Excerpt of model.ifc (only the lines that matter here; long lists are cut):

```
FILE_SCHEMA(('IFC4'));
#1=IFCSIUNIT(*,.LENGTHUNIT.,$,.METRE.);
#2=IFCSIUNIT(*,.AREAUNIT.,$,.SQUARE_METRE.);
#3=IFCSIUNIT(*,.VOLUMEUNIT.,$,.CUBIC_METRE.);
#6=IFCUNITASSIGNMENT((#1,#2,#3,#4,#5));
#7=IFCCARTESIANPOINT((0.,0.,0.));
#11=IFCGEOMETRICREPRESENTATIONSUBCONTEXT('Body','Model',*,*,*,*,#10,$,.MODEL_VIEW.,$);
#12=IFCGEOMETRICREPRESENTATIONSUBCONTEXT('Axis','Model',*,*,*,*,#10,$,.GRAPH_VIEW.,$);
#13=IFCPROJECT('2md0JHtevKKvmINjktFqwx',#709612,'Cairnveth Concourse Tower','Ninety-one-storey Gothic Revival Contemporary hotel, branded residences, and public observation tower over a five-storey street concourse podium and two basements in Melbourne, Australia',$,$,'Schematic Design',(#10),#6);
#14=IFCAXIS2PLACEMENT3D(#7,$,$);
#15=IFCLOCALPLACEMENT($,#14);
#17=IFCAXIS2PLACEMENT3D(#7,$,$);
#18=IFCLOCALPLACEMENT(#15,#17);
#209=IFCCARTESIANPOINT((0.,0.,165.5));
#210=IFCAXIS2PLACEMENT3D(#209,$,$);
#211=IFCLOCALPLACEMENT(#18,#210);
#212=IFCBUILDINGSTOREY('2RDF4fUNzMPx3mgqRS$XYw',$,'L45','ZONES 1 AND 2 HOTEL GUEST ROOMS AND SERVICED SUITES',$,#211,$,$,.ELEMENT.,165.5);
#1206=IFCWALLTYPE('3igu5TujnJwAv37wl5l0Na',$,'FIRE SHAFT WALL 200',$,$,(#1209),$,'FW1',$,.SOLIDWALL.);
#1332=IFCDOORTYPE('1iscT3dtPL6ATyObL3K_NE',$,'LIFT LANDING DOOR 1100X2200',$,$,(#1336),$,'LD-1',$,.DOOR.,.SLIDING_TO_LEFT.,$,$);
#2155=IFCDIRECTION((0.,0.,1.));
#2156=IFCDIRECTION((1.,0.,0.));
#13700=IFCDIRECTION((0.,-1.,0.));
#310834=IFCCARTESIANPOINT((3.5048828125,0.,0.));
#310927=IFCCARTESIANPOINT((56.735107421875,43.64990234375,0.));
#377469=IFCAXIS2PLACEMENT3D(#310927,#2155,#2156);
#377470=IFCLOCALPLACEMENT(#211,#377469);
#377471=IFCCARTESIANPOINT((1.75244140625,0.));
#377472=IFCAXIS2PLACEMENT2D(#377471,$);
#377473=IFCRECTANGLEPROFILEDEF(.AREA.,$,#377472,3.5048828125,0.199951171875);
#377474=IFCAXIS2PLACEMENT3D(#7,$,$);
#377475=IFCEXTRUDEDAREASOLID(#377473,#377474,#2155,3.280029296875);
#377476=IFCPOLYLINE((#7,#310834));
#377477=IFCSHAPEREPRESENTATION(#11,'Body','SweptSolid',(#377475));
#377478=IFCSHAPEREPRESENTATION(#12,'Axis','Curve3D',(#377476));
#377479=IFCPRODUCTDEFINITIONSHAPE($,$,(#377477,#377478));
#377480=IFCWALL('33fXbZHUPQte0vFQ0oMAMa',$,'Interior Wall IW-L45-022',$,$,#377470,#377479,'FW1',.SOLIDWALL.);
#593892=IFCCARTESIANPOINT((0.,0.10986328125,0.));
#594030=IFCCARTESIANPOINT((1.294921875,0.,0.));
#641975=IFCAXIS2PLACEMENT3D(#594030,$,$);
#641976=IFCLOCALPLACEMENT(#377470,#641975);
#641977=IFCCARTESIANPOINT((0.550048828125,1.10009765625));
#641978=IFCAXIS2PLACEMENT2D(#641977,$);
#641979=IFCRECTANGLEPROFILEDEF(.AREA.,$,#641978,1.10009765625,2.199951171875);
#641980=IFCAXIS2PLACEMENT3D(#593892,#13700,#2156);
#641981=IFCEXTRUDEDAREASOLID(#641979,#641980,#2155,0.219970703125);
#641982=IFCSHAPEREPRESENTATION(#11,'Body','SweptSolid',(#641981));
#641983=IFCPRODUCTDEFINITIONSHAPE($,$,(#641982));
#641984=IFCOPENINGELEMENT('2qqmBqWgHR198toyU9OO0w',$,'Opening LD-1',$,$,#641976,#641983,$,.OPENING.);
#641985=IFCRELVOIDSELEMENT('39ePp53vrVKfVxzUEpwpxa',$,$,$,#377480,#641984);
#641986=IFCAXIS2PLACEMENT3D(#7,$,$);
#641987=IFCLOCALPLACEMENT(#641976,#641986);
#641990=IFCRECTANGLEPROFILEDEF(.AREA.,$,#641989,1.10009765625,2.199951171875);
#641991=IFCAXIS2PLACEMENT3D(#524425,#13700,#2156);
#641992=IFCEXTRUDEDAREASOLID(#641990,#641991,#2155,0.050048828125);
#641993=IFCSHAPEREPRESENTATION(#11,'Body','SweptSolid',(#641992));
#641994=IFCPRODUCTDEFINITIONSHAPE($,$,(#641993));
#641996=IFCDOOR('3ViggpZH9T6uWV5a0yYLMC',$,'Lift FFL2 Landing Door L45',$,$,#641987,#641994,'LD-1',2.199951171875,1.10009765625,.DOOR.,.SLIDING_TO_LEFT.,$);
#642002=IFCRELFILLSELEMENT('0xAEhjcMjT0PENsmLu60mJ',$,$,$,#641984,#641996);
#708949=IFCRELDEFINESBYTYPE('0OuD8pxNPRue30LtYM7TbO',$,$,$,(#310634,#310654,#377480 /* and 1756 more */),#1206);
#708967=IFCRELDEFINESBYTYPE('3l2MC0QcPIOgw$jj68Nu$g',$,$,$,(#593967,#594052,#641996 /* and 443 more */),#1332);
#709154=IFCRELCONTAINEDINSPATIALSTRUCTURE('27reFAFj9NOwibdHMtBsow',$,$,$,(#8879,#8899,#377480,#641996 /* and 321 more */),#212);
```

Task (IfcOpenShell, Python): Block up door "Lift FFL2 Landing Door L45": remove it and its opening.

```python
import ifcopenshell
import ifcopenshell.api.feature
import ifcopenshell.api.root
import ifcopenshell.geom
import ifcopenshell.util.shape

model = ifcopenshell.open("model.ifc")
settings = ifcopenshell.geom.settings()


def volume(element):
    """Net volume in cubic metres, openings subtracted."""
    shape = ifcopenshell.geom.create_shape(settings, element)
    return ifcopenshell.util.shape.get_volume(shape.geometry)


door = model.by_id(641996)
opening = door.FillsVoids[0].RelatingOpeningElement
wall = opening.VoidsElements[0].RelatingBuildingElement
before = volume(wall)

ifcopenshell.api.root.remove_product(model, product=door)
ifcopenshell.api.feature.remove_feature(model, feature=opening)

after = volume(wall)

print(f"wall volume {before:.3f} -> {after:.3f} m3")

model.write("model_updated.ifc")
```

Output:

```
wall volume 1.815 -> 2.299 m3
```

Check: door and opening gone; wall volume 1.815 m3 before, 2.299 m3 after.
